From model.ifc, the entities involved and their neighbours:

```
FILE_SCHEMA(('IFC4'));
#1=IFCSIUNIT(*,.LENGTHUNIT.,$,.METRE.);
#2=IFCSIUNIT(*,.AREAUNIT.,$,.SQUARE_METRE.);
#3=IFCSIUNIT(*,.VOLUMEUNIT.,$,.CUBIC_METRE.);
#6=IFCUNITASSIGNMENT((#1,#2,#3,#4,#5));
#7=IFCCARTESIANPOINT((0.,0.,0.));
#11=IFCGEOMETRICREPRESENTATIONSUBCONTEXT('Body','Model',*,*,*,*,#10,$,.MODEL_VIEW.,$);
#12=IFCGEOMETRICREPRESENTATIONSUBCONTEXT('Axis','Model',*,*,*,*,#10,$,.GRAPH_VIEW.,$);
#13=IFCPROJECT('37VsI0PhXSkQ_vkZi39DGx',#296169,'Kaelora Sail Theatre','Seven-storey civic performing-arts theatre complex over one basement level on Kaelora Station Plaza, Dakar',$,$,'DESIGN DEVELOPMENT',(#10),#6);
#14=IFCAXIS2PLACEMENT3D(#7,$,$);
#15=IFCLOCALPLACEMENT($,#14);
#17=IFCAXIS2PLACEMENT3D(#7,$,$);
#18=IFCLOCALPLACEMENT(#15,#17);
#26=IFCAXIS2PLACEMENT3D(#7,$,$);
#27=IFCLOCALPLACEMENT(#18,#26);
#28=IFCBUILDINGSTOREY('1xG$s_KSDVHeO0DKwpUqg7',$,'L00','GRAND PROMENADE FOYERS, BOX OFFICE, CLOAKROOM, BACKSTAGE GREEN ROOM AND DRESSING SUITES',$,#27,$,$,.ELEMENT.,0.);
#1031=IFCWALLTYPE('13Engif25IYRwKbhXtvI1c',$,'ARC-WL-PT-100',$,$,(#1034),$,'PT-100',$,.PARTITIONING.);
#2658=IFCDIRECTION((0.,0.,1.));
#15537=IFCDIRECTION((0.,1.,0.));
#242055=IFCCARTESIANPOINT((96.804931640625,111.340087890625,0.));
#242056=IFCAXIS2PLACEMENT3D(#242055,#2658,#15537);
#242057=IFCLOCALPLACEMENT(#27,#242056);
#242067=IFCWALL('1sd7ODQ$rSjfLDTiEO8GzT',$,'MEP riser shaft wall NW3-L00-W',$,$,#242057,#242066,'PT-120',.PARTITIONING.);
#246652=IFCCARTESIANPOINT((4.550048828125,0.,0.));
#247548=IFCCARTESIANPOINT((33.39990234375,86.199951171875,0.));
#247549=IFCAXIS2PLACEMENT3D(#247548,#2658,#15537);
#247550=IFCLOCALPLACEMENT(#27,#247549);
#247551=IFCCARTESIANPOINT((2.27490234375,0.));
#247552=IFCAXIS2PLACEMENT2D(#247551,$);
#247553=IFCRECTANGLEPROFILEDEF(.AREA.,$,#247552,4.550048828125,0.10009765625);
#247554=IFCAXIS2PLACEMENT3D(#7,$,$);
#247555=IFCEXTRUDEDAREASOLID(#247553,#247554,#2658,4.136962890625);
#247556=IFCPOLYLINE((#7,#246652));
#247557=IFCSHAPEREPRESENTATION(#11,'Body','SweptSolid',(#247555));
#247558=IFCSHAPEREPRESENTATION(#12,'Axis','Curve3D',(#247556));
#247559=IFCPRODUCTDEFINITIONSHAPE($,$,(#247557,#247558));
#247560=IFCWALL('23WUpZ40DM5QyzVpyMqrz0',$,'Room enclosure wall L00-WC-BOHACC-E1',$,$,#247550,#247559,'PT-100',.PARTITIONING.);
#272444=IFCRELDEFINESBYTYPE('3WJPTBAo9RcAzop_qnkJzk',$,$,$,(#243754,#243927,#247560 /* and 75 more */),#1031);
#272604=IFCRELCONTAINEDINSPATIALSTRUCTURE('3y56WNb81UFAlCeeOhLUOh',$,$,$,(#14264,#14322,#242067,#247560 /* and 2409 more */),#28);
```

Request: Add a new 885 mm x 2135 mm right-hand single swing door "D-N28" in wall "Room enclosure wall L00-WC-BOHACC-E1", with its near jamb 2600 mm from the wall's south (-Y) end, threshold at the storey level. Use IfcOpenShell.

```python
import numpy as np
import ifcopenshell
import ifcopenshell.api.feature
import ifcopenshell.api.geometry
import ifcopenshell.api.root
import ifcopenshell.api.spatial
import ifcopenshell.geom
import ifcopenshell.util.element
import ifcopenshell.util.placement
import ifcopenshell.util.representation
import ifcopenshell.util.shape
import ifcopenshell.util.unit

model = ifcopenshell.open("model.ifc")
unit_scale = ifcopenshell.util.unit.calculate_unit_scale(model)
settings = ifcopenshell.geom.settings()


def volume(element):
    """Net volume in cubic metres, openings subtracted."""
    shape = ifcopenshell.geom.create_shape(settings, element)
    return ifcopenshell.util.shape.get_volume(shape.geometry)


wall = model.by_id(247560)
storey = ifcopenshell.util.element.get_container(wall, ifc_class="IfcBuildingStorey")
context = ifcopenshell.util.representation.get_context(model, "Model", "Body", "MODEL_VIEW")
before = volume(wall)

width, height, from_end, sill = 0.885, 2.135, 2.6, 0.0  # metres

# The wall runs along its own X axis, and the end named is its -X end.
wall_shape = ifcopenshell.geom.create_shape(settings, wall)
x, y, z = ifcopenshell.util.shape.get_vertices(wall_shape.geometry).T
start = x.min() + from_end
face, thickness = float(y.min()), float(y.max() - y.min())
wall_matrix = ifcopenshell.util.placement.get_local_placement(wall.ObjectPlacement)
level = ifcopenshell.util.placement.get_local_placement(storey.ObjectPlacement)[2, 3]


def in_wall(x, y):
    """Placement at x, y metres in the wall's axes, at sill height."""
    matrix = wall_matrix.copy()
    matrix[:, 3] = wall_matrix @ np.array([x / unit_scale, y / unit_scale, 0.0, 1.0])
    matrix[2, 3] = level + sill / unit_scale
    return matrix


# Opening: a box that overshoots both wall faces by 50 mm.
opening = ifcopenshell.api.root.create_entity(model, ifc_class="IfcOpeningElement", predefined_type="OPENING")
box = ifcopenshell.api.geometry.add_wall_representation(
    model, context=context, length=width, height=height, thickness=thickness + 0.1
)
ifcopenshell.api.geometry.assign_representation(model, product=opening, representation=box)
ifcopenshell.api.geometry.edit_object_placement(model, product=opening, matrix=in_wall(start, face - 0.05), is_si=False)
ifcopenshell.api.feature.add_feature(model, feature=opening, element=wall)

door = ifcopenshell.api.root.create_entity(model, ifc_class="IfcDoor", name="D-N28", predefined_type="DOOR")
door.OverallWidth, door.OverallHeight = width / unit_scale, height / unit_scale
door.OperationType = "SINGLE_SWING_RIGHT"
body = ifcopenshell.api.geometry.add_door_representation(
    model,
    context=context,
    overall_width=door.OverallWidth,
    overall_height=door.OverallHeight,
    operation_type="SINGLE_SWING_RIGHT",
    lining_properties={"LiningDepth": thickness / unit_scale, "ThresholdDepth": thickness / unit_scale},
)
ifcopenshell.api.geometry.assign_representation(model, product=door, representation=body)
ifcopenshell.api.spatial.assign_container(model, products=[door], relating_structure=storey)
ifcopenshell.api.feature.add_filling(model, opening=opening, element=door)

# The lining spans the wall, so the door starts at the wall face.
ifcopenshell.api.geometry.edit_object_placement(model, product=door, matrix=in_wall(start, face), is_si=False)

after = volume(wall)

print(f"wall volume {before:.3f} -> {after:.3f} m3")

model.write("model_v2.ifc")
```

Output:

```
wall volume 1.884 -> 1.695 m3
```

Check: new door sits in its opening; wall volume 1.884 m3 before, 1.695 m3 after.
